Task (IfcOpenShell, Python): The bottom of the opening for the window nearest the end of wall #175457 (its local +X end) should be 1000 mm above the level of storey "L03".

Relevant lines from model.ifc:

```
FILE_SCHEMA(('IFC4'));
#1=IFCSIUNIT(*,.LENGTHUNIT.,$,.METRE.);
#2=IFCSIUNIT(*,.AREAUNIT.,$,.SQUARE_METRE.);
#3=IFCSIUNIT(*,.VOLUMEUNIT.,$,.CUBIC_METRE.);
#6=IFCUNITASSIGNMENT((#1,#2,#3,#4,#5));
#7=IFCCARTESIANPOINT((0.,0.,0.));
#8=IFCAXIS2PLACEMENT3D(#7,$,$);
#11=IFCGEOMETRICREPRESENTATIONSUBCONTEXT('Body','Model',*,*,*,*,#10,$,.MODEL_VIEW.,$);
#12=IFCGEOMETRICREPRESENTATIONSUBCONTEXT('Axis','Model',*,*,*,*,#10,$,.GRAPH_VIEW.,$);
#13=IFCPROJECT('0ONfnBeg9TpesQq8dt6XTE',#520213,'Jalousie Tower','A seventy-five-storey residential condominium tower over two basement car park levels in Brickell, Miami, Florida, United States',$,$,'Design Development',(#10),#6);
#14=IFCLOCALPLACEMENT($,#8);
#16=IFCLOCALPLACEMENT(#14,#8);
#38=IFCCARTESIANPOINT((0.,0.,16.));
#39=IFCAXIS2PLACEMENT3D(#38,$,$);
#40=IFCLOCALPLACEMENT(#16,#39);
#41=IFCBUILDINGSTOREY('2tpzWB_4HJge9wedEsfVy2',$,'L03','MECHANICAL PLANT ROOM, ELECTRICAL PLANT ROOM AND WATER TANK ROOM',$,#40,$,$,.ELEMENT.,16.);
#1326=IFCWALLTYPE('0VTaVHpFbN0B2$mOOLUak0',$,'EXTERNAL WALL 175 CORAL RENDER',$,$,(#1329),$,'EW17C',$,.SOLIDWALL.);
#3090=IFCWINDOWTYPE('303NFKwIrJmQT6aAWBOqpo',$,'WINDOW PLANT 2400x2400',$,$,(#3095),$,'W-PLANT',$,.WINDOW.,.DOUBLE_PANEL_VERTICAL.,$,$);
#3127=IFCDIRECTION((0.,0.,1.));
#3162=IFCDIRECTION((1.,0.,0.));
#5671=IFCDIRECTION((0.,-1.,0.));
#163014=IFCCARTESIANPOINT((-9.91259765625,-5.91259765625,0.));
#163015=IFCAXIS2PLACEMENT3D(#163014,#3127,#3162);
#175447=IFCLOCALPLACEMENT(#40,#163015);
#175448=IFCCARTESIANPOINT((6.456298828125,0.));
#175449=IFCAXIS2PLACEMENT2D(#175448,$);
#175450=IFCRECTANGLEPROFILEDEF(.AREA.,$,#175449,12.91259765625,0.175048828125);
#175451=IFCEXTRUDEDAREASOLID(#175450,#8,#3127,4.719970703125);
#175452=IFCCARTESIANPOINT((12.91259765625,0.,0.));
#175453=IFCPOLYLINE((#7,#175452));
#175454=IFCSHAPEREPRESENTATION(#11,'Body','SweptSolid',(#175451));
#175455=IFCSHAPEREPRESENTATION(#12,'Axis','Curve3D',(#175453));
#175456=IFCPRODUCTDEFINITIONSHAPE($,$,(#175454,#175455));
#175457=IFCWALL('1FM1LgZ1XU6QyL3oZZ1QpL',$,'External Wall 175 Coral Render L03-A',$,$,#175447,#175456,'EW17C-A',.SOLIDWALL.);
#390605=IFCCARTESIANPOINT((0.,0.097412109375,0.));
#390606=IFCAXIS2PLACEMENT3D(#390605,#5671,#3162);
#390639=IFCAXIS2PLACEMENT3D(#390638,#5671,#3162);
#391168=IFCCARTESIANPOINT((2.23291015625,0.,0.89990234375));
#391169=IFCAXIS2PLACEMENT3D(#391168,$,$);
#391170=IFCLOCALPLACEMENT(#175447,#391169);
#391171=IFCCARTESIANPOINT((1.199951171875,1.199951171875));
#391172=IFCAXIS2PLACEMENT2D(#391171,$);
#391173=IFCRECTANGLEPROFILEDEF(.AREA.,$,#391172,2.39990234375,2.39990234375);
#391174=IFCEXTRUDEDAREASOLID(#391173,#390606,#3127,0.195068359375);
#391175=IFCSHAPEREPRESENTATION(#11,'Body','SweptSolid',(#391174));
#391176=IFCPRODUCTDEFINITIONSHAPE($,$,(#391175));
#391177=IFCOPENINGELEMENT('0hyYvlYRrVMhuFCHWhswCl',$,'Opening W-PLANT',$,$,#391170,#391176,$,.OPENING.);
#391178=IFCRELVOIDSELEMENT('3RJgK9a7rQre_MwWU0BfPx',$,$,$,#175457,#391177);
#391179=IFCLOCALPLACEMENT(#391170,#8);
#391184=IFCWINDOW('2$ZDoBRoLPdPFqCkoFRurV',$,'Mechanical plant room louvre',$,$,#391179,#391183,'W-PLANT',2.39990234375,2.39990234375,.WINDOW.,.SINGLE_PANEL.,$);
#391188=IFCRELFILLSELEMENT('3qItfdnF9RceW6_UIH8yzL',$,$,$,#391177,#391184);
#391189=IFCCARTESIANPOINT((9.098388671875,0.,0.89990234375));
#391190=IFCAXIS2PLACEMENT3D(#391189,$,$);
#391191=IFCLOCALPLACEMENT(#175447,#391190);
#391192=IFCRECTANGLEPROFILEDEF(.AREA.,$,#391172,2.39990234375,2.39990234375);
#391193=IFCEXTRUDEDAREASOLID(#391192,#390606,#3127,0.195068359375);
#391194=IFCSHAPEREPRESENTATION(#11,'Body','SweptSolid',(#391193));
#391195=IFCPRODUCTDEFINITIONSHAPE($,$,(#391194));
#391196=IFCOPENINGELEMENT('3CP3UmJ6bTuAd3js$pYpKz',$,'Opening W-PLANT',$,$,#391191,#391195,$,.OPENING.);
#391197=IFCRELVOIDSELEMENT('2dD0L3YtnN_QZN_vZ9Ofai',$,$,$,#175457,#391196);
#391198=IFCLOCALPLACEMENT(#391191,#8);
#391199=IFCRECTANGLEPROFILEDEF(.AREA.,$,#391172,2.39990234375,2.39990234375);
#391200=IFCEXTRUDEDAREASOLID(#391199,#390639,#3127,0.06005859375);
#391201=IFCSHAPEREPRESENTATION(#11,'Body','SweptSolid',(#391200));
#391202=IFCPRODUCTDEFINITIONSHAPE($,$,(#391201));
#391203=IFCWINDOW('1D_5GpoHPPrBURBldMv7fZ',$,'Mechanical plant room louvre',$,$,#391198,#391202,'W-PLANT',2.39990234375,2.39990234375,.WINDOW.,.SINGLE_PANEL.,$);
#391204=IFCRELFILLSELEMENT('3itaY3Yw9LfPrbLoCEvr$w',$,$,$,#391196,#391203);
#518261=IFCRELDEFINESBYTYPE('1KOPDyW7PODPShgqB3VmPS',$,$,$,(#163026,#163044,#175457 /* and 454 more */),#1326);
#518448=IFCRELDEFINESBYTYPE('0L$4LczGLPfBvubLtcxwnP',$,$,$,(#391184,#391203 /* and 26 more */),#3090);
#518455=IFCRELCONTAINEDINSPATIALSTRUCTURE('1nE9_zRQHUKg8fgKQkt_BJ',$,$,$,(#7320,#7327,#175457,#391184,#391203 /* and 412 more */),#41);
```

```python
import numpy as np
import ifcopenshell
import ifcopenshell.api.geometry
import ifcopenshell.geom
import ifcopenshell.util.element
import ifcopenshell.util.placement
import ifcopenshell.util.shape
import ifcopenshell.util.unit

model = ifcopenshell.open("model.ifc")
unit_scale = ifcopenshell.util.unit.calculate_unit_scale(model)

window = model.by_id(391203)
opening = window.FillsVoids[0].RelatingOpeningElement
storey = ifcopenshell.util.element.get_container(window, ifc_class="IfcBuildingStorey")
level = ifcopenshell.util.placement.get_local_placement(storey.ObjectPlacement)[2, 3]

# The opening's origin need not be at the sill, so measure its lowest point.
shape = ifcopenshell.geom.create_shape(ifcopenshell.geom.settings(), opening)
bottom = ifcopenshell.util.shape.get_shape_bottom_elevation(shape, shape.geometry) / unit_scale
dz = level + 1.0 - bottom

shift = np.array([0.0, 0.0, dz])
# The window is placed relative to its opening, so it follows when the opening moves.
matrix = ifcopenshell.util.placement.get_local_placement(opening.ObjectPlacement)
matrix[:3, 3] += shift
ifcopenshell.api.geometry.edit_object_placement(
    model, product=opening, matrix=matrix, is_si=False, should_transform_children=True
)

print(f"moved by {dz * unit_scale:+.3f} m")

model.write("model_edited.ifc")
```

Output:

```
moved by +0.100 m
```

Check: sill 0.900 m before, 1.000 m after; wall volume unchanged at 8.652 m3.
